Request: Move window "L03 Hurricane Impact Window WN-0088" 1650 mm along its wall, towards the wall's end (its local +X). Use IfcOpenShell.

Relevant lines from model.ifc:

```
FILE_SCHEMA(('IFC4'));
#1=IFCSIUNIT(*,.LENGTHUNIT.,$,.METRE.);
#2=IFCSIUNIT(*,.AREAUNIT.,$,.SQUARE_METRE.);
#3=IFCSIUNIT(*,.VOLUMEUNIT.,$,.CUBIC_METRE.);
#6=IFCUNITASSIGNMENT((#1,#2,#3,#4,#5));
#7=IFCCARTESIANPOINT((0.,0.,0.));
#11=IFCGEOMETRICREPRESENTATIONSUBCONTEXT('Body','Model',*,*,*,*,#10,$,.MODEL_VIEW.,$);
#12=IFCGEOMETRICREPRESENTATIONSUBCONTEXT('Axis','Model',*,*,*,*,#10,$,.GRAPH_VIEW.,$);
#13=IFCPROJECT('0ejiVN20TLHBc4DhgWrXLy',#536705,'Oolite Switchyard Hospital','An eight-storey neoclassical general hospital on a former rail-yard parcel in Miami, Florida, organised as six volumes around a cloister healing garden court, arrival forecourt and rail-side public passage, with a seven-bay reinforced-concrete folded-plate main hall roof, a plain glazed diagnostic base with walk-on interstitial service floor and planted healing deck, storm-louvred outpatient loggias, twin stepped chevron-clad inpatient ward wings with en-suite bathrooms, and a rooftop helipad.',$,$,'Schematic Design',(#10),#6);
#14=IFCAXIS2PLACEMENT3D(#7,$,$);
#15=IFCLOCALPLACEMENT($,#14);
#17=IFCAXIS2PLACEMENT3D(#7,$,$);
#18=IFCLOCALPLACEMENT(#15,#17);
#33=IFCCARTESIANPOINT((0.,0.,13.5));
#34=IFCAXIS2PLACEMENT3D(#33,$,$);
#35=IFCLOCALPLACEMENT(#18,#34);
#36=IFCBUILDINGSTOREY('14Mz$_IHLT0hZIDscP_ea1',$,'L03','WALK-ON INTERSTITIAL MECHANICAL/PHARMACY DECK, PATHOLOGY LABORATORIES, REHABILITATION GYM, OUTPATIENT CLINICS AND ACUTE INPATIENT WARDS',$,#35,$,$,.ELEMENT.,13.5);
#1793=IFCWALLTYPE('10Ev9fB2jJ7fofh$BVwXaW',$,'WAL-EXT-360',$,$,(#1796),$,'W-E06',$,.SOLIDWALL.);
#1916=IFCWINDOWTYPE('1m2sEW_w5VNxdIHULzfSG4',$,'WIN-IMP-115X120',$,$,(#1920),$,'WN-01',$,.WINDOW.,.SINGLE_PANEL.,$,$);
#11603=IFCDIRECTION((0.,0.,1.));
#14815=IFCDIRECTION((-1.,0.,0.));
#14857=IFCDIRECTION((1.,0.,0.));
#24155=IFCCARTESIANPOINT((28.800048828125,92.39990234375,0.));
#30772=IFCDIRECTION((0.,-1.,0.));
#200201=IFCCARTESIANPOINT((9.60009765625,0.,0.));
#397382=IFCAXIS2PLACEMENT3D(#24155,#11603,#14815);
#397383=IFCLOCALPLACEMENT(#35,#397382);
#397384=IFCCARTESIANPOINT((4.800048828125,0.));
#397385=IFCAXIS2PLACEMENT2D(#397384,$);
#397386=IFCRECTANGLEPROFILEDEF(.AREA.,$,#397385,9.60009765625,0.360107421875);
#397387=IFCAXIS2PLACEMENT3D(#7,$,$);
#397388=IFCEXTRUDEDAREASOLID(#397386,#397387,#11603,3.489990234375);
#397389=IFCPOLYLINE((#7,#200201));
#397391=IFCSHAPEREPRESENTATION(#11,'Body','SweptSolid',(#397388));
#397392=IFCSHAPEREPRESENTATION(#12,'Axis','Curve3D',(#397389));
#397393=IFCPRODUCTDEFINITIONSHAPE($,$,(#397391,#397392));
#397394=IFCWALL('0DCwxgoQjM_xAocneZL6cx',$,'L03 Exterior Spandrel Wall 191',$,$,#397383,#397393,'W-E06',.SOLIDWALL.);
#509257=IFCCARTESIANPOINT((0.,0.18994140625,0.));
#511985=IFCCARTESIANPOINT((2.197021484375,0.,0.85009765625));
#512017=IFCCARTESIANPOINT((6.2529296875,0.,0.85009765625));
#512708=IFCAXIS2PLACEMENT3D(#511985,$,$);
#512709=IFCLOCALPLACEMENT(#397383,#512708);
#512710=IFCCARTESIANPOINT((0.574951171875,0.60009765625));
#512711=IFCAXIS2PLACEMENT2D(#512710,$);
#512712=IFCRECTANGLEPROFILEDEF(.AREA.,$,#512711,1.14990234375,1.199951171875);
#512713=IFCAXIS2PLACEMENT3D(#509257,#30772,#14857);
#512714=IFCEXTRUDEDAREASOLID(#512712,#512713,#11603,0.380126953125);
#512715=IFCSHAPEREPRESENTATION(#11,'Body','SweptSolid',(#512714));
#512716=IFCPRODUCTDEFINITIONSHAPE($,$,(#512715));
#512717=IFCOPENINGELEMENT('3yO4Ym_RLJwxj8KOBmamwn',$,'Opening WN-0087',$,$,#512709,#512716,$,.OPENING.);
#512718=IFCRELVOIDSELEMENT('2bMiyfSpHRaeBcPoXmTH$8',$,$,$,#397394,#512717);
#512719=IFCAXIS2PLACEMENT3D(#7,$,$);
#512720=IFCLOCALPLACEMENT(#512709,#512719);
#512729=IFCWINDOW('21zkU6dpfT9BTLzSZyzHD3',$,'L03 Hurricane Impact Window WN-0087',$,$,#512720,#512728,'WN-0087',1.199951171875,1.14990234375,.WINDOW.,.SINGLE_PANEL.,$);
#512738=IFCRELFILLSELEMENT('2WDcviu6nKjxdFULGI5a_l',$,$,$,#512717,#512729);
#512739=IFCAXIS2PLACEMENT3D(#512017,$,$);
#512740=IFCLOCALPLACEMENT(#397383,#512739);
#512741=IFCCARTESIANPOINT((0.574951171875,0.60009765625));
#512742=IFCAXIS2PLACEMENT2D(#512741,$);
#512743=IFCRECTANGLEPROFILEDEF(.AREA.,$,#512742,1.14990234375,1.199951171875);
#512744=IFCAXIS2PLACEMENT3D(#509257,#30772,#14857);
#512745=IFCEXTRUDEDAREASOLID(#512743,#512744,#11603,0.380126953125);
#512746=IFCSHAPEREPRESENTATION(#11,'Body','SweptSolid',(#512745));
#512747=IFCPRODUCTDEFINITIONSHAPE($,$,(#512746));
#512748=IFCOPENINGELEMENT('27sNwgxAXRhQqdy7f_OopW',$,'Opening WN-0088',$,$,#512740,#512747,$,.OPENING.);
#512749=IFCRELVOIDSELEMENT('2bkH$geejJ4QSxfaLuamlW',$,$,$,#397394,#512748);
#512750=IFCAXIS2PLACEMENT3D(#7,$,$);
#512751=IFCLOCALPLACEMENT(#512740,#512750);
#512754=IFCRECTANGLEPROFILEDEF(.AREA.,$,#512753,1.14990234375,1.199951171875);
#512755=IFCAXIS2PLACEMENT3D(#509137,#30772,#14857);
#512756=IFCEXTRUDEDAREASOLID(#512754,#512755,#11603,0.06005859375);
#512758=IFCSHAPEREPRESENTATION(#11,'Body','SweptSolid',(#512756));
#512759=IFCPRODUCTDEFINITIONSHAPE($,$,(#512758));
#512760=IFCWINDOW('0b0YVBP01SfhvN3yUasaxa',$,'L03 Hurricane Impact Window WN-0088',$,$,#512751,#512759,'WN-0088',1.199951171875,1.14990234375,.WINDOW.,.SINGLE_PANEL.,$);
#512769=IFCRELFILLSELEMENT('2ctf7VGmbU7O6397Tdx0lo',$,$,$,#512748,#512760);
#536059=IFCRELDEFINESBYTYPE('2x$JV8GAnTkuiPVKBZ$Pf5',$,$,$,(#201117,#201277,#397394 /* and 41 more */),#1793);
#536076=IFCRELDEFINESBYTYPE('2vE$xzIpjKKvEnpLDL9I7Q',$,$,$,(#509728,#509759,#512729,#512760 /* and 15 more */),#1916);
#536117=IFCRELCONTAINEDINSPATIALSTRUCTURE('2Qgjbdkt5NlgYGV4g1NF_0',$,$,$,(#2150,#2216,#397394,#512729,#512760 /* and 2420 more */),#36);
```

```python
import ifcopenshell
import ifcopenshell.api.geometry
import ifcopenshell.util.placement
import ifcopenshell.util.unit

model = ifcopenshell.open("model.ifc")
unit_scale = ifcopenshell.util.unit.calculate_unit_scale(model)

window = model.by_guid("0b0YVBP01SfhvN3yUasaxa")
opening = window.FillsVoids[0].RelatingOpeningElement
wall = opening.VoidsElements[0].RelatingBuildingElement

wall_matrix = ifcopenshell.util.placement.get_local_placement(wall.ObjectPlacement)
shift = wall_matrix[:3, 0] * 1.65 / unit_scale
before = ifcopenshell.util.placement.get_local_placement(window.ObjectPlacement)[:3, 3].copy()

# The window is placed relative to its opening, so it follows when the opening moves.
matrix = ifcopenshell.util.placement.get_local_placement(opening.ObjectPlacement)
matrix[:3, 3] += shift
ifcopenshell.api.geometry.edit_object_placement(
    model, product=opening, matrix=matrix, is_si=False, should_transform_children=True
)

after = ifcopenshell.util.placement.get_local_placement(window.ObjectPlacement)[:3, 3]
print("window moved by", (after - before).round(3) + 0.0)

model.write("model_edited.ifc")
```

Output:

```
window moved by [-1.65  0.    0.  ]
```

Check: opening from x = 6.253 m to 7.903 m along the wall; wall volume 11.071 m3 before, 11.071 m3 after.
